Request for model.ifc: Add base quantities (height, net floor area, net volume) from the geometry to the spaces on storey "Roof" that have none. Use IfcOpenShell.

First a look at what the model holds.

```python
import ifcopenshell
import ifcopenshell.util.element
import ifcopenshell.util.unit

model = ifcopenshell.open("model.ifc")
print(model.schema)
for unit_type in ("LENGTHUNIT", "AREAUNIT", "VOLUMEUNIT"):
    print(unit_type, ifcopenshell.util.unit.calculate_unit_scale(model, unit_type))
storey = next(s for s in model.by_type("IfcBuildingStorey") if s.Name == "Roof")
spaces = [e for e in ifcopenshell.util.element.get_decomposition(storey) if e.is_a("IfcSpace")]
for e in sorted(spaces, key=lambda e: e.id()):
    print(e.id(), e.is_a(), e.Name, list(ifcopenshell.util.element.get_psets(e, qtos_only=True)), sep=" | ")
```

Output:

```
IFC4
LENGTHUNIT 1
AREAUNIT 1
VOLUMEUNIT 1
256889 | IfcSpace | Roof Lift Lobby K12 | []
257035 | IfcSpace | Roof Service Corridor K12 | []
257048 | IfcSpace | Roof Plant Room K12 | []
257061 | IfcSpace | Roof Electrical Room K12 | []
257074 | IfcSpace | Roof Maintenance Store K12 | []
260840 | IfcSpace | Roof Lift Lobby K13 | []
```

```python
import ifcopenshell
import ifcopenshell.api.pset
import ifcopenshell.geom
import ifcopenshell.util.element
import ifcopenshell.util.shape
import ifcopenshell.util.unit

model = ifcopenshell.open("model.ifc")
unit_scale = ifcopenshell.util.unit.calculate_unit_scale(model)
area_scale = ifcopenshell.util.unit.calculate_unit_scale(model, "AREAUNIT")
volume_scale = ifcopenshell.util.unit.calculate_unit_scale(model, "VOLUMEUNIT")
settings = ifcopenshell.geom.settings()

storey = next(s for s in model.by_type("IfcBuildingStorey") if s.Name == "Roof")
spaces = [e for e in ifcopenshell.util.element.get_decomposition(storey) if e.is_a("IfcSpace")]

for e in sorted(spaces, key=lambda e: e.id()):
    if ifcopenshell.util.element.get_psets(e, qtos_only=True, should_inherit=False):
        continue
    # Geometry comes back in metres, in the element's own axes.
    shape = ifcopenshell.geom.create_shape(settings, e)
    values = {
        "Height": ifcopenshell.util.shape.get_z(shape.geometry) / unit_scale,
        "NetFloorArea": ifcopenshell.util.shape.get_footprint_area(shape.geometry) / area_scale,
        "NetVolume": ifcopenshell.util.shape.get_volume(shape.geometry) / volume_scale,
    }
    qto = ifcopenshell.api.pset.add_qto(model, product=e, name="Qto_SpaceBaseQuantities")
    ifcopenshell.api.pset.edit_qto(model, qto=qto, properties=values)
    print(e.id(), {k: round(v, 3) for k, v in values.items()})

model.write("model_updated.ifc")
```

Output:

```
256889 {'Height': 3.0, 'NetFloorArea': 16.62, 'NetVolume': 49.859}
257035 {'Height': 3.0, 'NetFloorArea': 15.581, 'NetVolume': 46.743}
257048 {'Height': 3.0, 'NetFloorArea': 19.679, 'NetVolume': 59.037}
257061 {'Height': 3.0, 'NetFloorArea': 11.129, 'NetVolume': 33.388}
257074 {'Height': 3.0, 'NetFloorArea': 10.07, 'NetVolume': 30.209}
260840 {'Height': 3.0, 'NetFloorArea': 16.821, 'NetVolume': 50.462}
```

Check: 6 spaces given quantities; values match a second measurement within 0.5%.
